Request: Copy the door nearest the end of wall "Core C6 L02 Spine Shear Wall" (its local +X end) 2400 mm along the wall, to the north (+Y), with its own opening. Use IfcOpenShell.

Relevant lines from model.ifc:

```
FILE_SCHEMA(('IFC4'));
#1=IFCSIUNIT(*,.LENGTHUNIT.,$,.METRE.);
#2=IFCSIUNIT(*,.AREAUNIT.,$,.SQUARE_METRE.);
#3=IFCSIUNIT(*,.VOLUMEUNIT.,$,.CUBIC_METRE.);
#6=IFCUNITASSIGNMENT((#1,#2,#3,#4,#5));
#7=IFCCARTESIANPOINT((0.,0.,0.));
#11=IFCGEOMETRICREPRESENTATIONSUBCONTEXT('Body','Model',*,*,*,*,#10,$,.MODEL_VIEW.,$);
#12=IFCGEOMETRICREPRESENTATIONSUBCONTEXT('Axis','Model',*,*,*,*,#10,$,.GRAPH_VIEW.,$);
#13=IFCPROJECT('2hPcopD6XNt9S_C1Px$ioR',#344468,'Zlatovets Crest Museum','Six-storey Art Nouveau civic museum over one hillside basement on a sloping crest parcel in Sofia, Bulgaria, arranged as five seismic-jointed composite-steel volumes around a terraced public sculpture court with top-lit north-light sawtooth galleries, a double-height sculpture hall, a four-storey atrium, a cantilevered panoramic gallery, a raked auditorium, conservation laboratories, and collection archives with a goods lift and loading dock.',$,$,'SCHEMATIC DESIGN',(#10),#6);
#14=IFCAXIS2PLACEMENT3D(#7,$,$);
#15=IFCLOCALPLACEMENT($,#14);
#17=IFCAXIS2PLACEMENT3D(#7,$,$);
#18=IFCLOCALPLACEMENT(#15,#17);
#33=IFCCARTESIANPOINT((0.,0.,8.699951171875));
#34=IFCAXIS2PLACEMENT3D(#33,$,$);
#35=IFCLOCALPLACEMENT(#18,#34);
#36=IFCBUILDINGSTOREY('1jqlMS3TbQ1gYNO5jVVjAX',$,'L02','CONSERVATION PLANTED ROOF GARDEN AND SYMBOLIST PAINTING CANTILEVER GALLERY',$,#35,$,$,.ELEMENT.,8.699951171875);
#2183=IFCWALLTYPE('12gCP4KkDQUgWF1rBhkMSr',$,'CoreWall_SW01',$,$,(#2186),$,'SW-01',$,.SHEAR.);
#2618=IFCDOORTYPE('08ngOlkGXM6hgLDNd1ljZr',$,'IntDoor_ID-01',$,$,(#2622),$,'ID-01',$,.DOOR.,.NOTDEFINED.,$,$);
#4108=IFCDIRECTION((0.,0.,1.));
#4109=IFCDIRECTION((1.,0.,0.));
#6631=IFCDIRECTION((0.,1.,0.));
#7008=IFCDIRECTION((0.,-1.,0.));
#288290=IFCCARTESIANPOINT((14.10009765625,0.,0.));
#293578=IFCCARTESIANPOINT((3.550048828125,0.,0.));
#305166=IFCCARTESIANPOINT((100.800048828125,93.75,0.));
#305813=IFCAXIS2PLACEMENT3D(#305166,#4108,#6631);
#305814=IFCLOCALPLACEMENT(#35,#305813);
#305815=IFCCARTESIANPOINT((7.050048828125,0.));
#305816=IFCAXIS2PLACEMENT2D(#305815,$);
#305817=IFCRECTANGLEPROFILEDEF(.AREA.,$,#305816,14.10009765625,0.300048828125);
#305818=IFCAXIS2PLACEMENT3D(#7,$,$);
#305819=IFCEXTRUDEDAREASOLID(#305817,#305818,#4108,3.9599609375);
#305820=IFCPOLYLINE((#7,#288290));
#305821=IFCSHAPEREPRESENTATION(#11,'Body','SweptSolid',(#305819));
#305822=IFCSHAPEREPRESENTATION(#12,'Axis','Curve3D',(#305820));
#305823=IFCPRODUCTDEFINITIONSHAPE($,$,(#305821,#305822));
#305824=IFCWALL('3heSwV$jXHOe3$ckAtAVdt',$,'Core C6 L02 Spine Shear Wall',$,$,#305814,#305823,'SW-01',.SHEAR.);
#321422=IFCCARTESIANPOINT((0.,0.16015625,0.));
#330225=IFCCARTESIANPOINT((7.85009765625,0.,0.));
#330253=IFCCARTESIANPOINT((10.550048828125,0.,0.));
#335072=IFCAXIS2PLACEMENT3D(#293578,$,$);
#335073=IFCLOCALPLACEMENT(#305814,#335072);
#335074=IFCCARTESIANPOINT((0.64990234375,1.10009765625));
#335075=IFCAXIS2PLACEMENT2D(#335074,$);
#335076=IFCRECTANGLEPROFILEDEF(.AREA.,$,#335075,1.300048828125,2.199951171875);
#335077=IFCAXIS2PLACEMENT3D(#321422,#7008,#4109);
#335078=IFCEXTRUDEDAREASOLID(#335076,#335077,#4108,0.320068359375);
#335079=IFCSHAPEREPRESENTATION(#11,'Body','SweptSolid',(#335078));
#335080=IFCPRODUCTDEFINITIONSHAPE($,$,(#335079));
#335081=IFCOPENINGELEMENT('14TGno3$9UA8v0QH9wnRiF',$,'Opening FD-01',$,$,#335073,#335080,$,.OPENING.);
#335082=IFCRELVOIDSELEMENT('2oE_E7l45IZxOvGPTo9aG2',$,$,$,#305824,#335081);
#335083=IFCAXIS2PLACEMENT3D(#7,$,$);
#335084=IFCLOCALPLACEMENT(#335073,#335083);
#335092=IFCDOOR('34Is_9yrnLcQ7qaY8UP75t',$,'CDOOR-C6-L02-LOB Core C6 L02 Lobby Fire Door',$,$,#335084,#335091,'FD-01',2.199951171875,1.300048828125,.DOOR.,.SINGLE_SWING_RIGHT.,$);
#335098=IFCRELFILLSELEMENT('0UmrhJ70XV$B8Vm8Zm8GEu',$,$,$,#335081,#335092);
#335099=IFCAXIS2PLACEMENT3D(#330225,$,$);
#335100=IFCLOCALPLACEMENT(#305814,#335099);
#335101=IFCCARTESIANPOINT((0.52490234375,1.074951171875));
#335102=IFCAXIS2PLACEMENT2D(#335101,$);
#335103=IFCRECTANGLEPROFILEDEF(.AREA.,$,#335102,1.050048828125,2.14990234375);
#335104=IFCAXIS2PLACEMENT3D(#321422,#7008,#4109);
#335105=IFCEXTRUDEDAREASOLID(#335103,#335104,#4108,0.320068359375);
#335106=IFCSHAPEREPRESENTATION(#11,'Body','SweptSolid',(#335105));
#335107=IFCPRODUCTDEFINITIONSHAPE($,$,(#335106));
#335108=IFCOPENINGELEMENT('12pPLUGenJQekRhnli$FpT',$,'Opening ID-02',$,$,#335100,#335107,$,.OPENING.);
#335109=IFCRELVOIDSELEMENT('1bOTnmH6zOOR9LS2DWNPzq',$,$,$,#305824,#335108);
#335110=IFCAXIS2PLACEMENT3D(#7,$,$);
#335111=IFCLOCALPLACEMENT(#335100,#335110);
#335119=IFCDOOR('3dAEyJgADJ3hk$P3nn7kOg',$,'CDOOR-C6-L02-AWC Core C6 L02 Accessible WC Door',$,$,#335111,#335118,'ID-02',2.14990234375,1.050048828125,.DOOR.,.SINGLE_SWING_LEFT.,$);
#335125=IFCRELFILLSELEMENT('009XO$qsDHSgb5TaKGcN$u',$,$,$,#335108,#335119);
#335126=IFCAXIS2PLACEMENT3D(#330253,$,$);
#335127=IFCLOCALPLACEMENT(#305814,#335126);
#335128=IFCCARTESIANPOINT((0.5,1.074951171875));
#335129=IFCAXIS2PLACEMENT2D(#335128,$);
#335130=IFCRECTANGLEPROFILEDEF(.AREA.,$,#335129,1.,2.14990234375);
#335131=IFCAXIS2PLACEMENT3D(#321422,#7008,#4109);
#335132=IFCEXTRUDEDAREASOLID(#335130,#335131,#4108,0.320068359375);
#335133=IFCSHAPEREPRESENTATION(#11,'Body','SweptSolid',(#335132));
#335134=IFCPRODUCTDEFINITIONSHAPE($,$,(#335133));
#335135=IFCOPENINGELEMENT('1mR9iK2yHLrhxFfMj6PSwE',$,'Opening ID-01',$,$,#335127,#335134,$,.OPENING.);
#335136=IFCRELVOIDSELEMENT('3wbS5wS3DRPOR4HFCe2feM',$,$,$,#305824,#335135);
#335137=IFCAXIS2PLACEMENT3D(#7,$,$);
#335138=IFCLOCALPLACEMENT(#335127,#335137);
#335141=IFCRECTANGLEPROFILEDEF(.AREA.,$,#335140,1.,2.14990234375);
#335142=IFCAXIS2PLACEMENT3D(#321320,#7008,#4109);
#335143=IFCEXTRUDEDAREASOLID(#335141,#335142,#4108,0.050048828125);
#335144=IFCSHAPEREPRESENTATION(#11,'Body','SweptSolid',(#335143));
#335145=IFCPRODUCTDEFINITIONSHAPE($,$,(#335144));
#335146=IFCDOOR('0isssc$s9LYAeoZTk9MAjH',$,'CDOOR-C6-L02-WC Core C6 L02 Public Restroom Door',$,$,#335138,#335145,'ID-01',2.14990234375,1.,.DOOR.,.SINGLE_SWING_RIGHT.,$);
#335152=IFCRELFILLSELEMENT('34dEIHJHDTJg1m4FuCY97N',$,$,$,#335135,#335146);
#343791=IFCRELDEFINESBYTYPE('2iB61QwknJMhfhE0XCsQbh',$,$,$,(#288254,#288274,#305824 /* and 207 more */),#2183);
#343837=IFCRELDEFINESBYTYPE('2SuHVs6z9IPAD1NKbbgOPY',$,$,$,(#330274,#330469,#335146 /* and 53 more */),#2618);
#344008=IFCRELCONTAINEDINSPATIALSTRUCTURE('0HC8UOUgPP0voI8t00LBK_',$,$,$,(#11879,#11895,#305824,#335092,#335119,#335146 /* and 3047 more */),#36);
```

```python
import ifcopenshell
import ifcopenshell.api.feature
import ifcopenshell.api.geometry
import ifcopenshell.api.root
import ifcopenshell.geom
import ifcopenshell.util.element
import ifcopenshell.util.placement
import ifcopenshell.util.shape

model = ifcopenshell.open("model.ifc")
settings = ifcopenshell.geom.settings()


def volume(element):
    """Net volume in cubic metres, openings subtracted."""
    shape = ifcopenshell.geom.create_shape(settings, element)
    return ifcopenshell.util.shape.get_volume(shape.geometry)


door = model.by_guid("0isssc$s9LYAeoZTk9MAjH")
opening = door.FillsVoids[0].RelatingOpeningElement
wall = opening.VoidsElements[0].RelatingBuildingElement
before = volume(wall)
shift = ifcopenshell.util.placement.get_local_placement(wall.ObjectPlacement)[:3, 0] * 2.4

# copy_class copies the void relationship, type, container and properties, but no geometry.
new_opening = ifcopenshell.api.root.copy_class(model, product=opening)
new_opening.Representation = ifcopenshell.util.element.copy_deep(
    model, opening.Representation, exclude=["IfcGeometricRepresentationContext", "IfcRepresentationMap"]
)
new_door = ifcopenshell.api.root.copy_class(model, product=door)
new_door.Representation = ifcopenshell.util.element.copy_deep(
    model, door.Representation, exclude=["IfcGeometricRepresentationContext", "IfcRepresentationMap"]
)
new_door.Tag = None
ifcopenshell.api.feature.add_filling(model, opening=new_opening, element=new_door)

for old, new in ((opening, new_opening), (door, new_door)):
    matrix = ifcopenshell.util.placement.get_local_placement(old.ObjectPlacement)
    matrix[:3, 3] += shift
    ifcopenshell.api.geometry.edit_object_placement(model, product=new, matrix=matrix, is_si=False)

after = volume(wall)

print(f"wall volume {before:.3f} -> {after:.3f} m3")

model.write("model_rev.ifc")
```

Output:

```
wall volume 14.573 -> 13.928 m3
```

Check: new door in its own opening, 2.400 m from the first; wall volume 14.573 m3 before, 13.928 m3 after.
